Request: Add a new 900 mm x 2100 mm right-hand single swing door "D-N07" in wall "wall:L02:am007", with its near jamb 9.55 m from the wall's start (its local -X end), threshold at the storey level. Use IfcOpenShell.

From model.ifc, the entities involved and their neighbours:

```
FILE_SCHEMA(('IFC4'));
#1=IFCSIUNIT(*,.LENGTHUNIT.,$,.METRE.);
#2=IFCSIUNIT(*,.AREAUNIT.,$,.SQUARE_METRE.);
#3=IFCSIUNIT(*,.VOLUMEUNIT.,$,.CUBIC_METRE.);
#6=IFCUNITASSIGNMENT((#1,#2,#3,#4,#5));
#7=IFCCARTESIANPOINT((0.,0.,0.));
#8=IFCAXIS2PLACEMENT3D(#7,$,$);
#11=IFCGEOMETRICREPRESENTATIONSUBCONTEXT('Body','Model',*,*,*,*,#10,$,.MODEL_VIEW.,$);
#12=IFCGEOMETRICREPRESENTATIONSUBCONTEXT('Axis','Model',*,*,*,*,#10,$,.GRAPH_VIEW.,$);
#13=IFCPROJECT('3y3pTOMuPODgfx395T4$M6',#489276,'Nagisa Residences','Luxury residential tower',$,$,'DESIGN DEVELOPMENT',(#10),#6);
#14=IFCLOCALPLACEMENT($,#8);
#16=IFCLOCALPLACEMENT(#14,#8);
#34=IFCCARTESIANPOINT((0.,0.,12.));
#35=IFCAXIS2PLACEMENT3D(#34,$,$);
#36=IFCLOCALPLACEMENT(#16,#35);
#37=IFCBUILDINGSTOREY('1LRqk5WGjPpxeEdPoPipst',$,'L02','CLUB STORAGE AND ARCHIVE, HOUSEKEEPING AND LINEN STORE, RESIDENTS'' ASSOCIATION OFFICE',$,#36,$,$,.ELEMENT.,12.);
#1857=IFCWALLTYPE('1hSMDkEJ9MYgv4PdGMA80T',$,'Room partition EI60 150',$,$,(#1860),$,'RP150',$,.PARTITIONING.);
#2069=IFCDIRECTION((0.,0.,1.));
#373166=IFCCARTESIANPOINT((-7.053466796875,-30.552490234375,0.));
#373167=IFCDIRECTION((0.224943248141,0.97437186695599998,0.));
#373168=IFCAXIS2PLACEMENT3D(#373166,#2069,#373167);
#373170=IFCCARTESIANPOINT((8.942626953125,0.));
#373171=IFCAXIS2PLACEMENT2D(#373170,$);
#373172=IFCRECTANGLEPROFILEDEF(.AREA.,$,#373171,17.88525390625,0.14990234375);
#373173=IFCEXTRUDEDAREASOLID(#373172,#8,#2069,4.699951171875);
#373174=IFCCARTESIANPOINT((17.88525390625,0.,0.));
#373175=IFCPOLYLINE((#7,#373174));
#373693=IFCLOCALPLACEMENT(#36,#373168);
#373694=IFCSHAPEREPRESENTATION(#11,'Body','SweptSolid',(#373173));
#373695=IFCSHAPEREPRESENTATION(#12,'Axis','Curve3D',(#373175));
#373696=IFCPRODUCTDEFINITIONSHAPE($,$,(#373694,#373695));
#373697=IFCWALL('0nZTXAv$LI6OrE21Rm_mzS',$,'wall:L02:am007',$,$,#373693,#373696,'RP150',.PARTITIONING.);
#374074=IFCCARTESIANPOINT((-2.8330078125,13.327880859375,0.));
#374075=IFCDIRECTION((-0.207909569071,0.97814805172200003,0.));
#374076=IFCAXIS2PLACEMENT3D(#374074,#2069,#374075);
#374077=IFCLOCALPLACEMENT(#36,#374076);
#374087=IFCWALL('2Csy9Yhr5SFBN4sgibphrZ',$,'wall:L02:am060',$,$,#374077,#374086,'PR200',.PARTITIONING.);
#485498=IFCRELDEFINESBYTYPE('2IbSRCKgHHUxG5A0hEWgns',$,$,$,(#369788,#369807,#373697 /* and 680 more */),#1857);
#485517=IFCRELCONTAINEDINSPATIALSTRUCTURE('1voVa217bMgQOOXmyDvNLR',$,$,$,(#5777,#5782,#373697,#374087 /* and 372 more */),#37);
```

```python
import numpy as np
import ifcopenshell
import ifcopenshell.api.feature
import ifcopenshell.api.geometry
import ifcopenshell.api.root
import ifcopenshell.api.spatial
import ifcopenshell.geom
import ifcopenshell.util.element
import ifcopenshell.util.placement
import ifcopenshell.util.representation
import ifcopenshell.util.shape
import ifcopenshell.util.unit

model = ifcopenshell.open("model.ifc")
unit_scale = ifcopenshell.util.unit.calculate_unit_scale(model)
settings = ifcopenshell.geom.settings()


def volume(element):
    """Net volume in cubic metres, openings subtracted."""
    shape = ifcopenshell.geom.create_shape(settings, element)
    return ifcopenshell.util.shape.get_volume(shape.geometry)


wall = model.by_id(373697)
storey = ifcopenshell.util.element.get_container(wall, ifc_class="IfcBuildingStorey")
context = ifcopenshell.util.representation.get_context(model, "Model", "Body", "MODEL_VIEW")
before = volume(wall)

width, height, from_end, sill = 0.9, 2.1, 9.55, 0.0  # metres

# The wall runs along its own X axis, and the end named is its -X end.
wall_shape = ifcopenshell.geom.create_shape(settings, wall)
x, y, z = ifcopenshell.util.shape.get_vertices(wall_shape.geometry).T
start = x.min() + from_end
face, thickness = float(y.min()), float(y.max() - y.min())
wall_matrix = ifcopenshell.util.placement.get_local_placement(wall.ObjectPlacement)
level = ifcopenshell.util.placement.get_local_placement(storey.ObjectPlacement)[2, 3]


def in_wall(x, y):
    """Placement at x, y metres in the wall's axes, at sill height."""
    matrix = wall_matrix.copy()
    matrix[:, 3] = wall_matrix @ np.array([x / unit_scale, y / unit_scale, 0.0, 1.0])
    matrix[2, 3] = level + sill / unit_scale
    return matrix


# Opening: a box that overshoots both wall faces by 50 mm.
opening = ifcopenshell.api.root.create_entity(model, ifc_class="IfcOpeningElement", predefined_type="OPENING")
box = ifcopenshell.api.geometry.add_wall_representation(
    model, context=context, length=width, height=height, thickness=thickness + 0.1
)
ifcopenshell.api.geometry.assign_representation(model, product=opening, representation=box)
ifcopenshell.api.geometry.edit_object_placement(model, product=opening, matrix=in_wall(start, face - 0.05), is_si=False)
ifcopenshell.api.feature.add_feature(model, feature=opening, element=wall)

door = ifcopenshell.api.root.create_entity(model, ifc_class="IfcDoor", name="D-N07", predefined_type="DOOR")
door.OverallWidth, door.OverallHeight = width / unit_scale, height / unit_scale
door.OperationType = "SINGLE_SWING_RIGHT"
body = ifcopenshell.api.geometry.add_door_representation(
    model,
    context=context,
    overall_width=door.OverallWidth,
    overall_height=door.OverallHeight,
    operation_type="SINGLE_SWING_RIGHT",
    lining_properties={"LiningDepth": thickness / unit_scale, "ThresholdDepth": thickness / unit_scale},
)
ifcopenshell.api.geometry.assign_representation(model, product=door, representation=body)
ifcopenshell.api.spatial.assign_container(model, products=[door], relating_structure=storey)
ifcopenshell.api.feature.add_filling(model, opening=opening, element=door)

# The lining spans the wall, so the door starts at the wall face.
ifcopenshell.api.geometry.edit_object_placement(model, product=door, matrix=in_wall(start, face), is_si=False)

after = volume(wall)

print(f"wall volume {before:.3f} -> {after:.3f} m3")

model.write("model_rev.ifc")
```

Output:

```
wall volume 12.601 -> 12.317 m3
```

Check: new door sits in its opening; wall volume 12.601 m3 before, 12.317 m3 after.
